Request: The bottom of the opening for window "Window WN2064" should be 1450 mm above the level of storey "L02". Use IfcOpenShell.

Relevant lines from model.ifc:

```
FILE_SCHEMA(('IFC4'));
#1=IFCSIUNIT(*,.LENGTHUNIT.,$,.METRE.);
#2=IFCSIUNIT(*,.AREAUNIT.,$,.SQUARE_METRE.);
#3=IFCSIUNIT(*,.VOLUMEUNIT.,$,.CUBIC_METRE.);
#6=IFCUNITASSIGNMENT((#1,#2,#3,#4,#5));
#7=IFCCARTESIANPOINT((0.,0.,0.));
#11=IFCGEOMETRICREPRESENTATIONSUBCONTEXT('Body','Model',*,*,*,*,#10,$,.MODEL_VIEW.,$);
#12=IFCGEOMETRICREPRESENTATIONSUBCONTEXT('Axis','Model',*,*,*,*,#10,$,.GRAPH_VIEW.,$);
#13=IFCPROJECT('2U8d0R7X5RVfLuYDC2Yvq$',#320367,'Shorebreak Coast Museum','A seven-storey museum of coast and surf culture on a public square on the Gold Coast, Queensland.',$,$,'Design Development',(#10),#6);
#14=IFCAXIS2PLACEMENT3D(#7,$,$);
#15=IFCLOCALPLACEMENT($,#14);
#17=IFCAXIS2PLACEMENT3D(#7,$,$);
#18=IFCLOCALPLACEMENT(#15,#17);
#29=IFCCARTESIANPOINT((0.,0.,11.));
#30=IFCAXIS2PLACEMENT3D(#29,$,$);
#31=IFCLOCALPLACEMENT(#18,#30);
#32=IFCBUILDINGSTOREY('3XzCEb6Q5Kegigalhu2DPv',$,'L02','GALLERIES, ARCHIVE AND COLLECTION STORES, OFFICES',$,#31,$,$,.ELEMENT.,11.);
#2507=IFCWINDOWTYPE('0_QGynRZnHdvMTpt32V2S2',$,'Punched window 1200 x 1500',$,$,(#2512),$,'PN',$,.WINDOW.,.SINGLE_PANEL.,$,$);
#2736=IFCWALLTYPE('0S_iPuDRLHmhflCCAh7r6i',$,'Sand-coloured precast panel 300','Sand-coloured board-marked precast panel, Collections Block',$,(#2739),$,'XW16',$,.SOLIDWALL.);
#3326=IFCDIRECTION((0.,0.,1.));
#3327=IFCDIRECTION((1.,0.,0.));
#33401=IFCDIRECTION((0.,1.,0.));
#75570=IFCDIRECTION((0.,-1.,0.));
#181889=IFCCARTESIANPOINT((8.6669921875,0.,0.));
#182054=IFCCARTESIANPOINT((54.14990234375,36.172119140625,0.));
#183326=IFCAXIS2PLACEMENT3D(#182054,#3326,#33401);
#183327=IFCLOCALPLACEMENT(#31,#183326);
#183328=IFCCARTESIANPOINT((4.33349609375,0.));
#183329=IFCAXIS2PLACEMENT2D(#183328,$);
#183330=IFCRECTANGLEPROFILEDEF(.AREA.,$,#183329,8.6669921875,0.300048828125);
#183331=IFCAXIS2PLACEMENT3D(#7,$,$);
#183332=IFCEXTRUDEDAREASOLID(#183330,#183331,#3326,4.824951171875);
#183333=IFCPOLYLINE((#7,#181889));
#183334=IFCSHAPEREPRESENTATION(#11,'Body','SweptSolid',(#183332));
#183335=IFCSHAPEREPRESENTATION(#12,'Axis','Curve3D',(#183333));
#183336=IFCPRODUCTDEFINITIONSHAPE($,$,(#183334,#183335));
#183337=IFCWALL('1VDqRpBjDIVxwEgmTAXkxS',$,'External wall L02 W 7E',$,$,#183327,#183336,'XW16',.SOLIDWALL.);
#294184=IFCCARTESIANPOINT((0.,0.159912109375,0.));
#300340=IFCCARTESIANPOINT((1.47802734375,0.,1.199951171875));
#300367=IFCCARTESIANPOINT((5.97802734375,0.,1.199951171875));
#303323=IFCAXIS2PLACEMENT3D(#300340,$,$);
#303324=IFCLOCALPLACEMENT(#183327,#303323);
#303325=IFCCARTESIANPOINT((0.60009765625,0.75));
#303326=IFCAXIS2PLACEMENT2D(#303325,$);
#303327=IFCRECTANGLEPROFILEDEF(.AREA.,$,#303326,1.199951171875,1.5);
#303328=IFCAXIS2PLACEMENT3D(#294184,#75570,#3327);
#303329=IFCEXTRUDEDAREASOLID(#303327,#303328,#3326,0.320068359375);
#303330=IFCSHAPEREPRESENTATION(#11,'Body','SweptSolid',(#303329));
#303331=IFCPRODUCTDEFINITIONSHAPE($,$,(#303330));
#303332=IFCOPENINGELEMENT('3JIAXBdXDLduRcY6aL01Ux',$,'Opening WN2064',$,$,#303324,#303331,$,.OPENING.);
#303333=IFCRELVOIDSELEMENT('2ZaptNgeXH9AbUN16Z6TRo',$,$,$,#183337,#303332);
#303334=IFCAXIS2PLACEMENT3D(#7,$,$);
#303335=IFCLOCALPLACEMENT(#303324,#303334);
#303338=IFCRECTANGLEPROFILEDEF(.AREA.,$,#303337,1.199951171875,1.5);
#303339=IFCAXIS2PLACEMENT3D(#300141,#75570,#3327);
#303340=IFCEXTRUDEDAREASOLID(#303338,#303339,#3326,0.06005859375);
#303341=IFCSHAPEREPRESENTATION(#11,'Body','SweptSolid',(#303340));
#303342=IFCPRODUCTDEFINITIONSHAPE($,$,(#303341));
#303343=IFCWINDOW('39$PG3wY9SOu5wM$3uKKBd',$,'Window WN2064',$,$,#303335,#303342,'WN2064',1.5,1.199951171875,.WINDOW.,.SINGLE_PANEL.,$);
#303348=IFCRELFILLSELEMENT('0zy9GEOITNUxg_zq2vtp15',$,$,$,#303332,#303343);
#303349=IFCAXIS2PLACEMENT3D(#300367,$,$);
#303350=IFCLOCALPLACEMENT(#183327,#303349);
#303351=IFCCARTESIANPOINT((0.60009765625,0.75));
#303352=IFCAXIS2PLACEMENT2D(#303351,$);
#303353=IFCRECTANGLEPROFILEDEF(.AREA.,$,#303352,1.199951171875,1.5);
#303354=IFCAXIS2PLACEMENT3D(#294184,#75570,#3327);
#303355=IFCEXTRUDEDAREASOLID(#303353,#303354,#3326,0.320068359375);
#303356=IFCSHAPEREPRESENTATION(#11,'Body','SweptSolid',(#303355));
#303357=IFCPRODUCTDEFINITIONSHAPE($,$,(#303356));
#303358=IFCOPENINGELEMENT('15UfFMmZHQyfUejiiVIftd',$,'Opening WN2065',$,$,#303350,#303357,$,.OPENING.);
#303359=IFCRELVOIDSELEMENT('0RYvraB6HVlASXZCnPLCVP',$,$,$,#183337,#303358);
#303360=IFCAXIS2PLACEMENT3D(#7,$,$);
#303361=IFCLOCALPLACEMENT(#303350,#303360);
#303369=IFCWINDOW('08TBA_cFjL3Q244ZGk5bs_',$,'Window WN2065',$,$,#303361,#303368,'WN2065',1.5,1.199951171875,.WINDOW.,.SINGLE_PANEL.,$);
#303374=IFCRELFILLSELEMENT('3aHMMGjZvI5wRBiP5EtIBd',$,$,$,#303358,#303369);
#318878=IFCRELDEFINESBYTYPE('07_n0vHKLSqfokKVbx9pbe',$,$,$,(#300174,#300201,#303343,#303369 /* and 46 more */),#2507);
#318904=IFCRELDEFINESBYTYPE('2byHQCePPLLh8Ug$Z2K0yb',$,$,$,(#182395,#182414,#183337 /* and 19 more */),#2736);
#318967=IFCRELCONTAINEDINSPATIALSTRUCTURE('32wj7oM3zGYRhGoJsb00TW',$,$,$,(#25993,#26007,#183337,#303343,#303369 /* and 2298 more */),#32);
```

```python
import numpy as np
import ifcopenshell
import ifcopenshell.api.geometry
import ifcopenshell.geom
import ifcopenshell.util.element
import ifcopenshell.util.placement
import ifcopenshell.util.shape
import ifcopenshell.util.unit

model = ifcopenshell.open("model.ifc")
unit_scale = ifcopenshell.util.unit.calculate_unit_scale(model)

window = model.by_guid("39$PG3wY9SOu5wM$3uKKBd")
opening = window.FillsVoids[0].RelatingOpeningElement
storey = ifcopenshell.util.element.get_container(window, ifc_class="IfcBuildingStorey")
level = ifcopenshell.util.placement.get_local_placement(storey.ObjectPlacement)[2, 3]

# The opening's origin need not be at the sill, so measure its lowest point.
shape = ifcopenshell.geom.create_shape(ifcopenshell.geom.settings(), opening)
bottom = ifcopenshell.util.shape.get_shape_bottom_elevation(shape, shape.geometry) / unit_scale
dz = level + 1.45 - bottom

shift = np.array([0.0, 0.0, dz])
# The window is placed relative to its opening, so it follows when the opening moves.
matrix = ifcopenshell.util.placement.get_local_placement(opening.ObjectPlacement)
matrix[:3, 3] += shift
ifcopenshell.api.geometry.edit_object_placement(
    model, product=opening, matrix=matrix, is_si=False, should_transform_children=True
)

print(f"moved by {dz * unit_scale:+.3f} m")

model.write("model_rev.ifc")
```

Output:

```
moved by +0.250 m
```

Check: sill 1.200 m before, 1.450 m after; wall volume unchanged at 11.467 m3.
